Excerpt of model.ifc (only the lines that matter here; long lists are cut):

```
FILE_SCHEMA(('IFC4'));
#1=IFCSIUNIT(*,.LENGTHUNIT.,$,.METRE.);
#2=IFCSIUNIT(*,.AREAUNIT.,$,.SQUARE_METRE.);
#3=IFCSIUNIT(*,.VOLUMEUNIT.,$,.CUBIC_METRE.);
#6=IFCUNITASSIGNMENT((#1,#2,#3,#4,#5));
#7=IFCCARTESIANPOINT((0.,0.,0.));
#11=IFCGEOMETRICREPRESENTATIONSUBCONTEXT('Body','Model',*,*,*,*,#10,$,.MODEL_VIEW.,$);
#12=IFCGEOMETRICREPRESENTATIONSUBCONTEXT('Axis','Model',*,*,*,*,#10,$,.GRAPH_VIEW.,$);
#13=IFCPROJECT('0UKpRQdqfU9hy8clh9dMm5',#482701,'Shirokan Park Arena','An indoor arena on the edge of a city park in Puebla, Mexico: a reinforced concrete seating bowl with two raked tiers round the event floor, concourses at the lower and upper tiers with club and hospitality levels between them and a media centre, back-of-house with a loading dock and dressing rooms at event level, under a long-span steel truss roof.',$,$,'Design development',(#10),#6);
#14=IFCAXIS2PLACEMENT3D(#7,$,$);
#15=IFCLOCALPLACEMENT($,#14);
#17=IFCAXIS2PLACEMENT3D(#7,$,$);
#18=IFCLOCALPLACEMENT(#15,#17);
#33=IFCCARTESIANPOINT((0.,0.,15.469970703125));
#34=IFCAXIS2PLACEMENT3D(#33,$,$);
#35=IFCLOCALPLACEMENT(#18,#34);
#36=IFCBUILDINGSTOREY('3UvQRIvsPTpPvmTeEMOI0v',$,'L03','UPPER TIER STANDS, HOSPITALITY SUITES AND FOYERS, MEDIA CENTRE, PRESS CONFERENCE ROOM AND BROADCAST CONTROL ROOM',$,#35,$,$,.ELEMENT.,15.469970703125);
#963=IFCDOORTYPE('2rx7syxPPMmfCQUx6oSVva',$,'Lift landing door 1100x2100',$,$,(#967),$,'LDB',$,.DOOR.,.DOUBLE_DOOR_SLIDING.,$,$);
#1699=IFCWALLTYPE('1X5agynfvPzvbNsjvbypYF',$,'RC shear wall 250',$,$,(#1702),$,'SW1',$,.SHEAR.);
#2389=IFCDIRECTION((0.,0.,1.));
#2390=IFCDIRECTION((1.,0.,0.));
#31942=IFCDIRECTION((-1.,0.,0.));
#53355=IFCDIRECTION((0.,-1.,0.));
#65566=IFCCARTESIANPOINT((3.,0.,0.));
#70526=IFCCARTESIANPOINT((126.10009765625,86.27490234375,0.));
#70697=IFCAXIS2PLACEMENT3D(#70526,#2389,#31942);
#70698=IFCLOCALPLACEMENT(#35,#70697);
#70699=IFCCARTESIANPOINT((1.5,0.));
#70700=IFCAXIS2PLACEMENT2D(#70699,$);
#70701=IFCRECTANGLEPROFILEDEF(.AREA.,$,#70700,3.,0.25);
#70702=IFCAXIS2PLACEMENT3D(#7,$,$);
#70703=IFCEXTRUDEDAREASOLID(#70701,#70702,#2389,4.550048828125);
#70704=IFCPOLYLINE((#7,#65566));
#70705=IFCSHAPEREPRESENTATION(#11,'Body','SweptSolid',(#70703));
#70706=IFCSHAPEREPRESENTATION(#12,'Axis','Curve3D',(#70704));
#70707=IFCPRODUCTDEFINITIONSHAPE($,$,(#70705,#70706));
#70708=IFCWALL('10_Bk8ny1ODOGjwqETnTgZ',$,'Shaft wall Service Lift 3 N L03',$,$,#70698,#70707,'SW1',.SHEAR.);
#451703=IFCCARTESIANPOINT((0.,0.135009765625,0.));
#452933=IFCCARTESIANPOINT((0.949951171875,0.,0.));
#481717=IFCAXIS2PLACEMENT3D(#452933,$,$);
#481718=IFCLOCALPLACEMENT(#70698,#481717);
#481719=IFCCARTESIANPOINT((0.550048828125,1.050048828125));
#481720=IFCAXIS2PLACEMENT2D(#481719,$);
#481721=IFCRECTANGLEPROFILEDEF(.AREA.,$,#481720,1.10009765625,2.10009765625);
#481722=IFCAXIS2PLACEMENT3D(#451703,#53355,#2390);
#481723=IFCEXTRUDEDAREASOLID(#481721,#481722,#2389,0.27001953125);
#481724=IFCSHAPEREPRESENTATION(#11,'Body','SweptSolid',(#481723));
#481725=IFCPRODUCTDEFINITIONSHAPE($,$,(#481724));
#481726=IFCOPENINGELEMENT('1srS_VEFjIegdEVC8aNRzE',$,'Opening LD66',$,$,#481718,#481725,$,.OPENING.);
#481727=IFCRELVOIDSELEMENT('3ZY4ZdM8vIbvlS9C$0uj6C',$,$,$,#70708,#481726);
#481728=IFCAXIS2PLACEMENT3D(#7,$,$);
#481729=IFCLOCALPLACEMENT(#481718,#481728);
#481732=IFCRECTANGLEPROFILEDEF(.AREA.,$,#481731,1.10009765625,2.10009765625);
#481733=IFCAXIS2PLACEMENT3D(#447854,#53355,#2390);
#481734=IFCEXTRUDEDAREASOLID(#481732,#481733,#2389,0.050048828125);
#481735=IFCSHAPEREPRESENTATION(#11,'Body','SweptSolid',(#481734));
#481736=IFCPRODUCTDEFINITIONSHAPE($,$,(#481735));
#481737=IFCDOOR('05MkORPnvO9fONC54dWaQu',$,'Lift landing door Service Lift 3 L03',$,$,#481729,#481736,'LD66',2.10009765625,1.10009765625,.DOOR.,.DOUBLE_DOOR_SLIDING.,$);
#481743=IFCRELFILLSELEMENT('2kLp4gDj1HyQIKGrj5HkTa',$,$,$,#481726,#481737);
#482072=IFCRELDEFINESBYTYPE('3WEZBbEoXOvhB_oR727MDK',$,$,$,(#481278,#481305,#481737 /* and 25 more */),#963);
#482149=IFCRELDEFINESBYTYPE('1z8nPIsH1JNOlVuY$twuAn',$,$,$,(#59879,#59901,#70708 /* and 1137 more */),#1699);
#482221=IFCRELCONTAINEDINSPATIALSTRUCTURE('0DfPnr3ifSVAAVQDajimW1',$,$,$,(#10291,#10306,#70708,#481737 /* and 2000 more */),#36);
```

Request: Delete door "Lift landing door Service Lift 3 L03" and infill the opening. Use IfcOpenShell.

```python
import ifcopenshell
import ifcopenshell.api.feature
import ifcopenshell.api.root
import ifcopenshell.geom
import ifcopenshell.util.shape

model = ifcopenshell.open("model.ifc")
settings = ifcopenshell.geom.settings()


def volume(element):
    """Net volume in cubic metres, openings subtracted."""
    shape = ifcopenshell.geom.create_shape(settings, element)
    return ifcopenshell.util.shape.get_volume(shape.geometry)


door = model.by_guid("05MkORPnvO9fONC54dWaQu")
opening = door.FillsVoids[0].RelatingOpeningElement
wall = opening.VoidsElements[0].RelatingBuildingElement
before = volume(wall)

ifcopenshell.api.root.remove_product(model, product=door)
ifcopenshell.api.feature.remove_feature(model, feature=opening)

after = volume(wall)

print(f"wall volume {before:.3f} -> {after:.3f} m3")

model.write("model_updated.ifc")
```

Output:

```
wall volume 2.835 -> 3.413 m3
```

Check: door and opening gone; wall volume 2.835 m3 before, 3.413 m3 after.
